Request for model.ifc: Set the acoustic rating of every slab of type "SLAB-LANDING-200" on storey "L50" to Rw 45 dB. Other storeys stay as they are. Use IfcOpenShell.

First a look at what the model holds.

```python
import ifcopenshell
import ifcopenshell.util.element

model = ifcopenshell.open("model.ifc")
print(model.schema)
storey = next(s for s in model.by_type("IfcBuildingStorey") if s.Name == "L50")
slabs = [e for e in ifcopenshell.util.element.get_decomposition(storey) if e.is_a("IfcSlab")]
seen = {}
for e in slabs:
    element_type = ifcopenshell.util.element.get_type(e)
    key = (element_type.Name if element_type != e and element_type else None, ifcopenshell.util.element.get_pset(e, "Pset_SlabCommon", "AcousticRating"))
    seen[key] = seen.get(key, 0) + 1
for (name, value), count in sorted(seen.items(), key=str):
    print(count, "x", name, "|", value)
```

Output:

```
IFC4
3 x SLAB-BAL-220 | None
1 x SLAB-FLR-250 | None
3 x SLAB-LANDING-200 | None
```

```python
import ifcopenshell
import ifcopenshell.api.pset
import ifcopenshell.util.element

model = ifcopenshell.open("model.ifc")

storey = next(s for s in model.by_type("IfcBuildingStorey") if s.Name == "L50")
slabs = [e for e in ifcopenshell.util.element.get_decomposition(storey) if e.is_a("IfcSlab")]

count = 0
for e in slabs:
    element_type = ifcopenshell.util.element.get_type(e)
    if element_type in (None, e) or element_type.Name != "SLAB-LANDING-200":
        continue
    found = ifcopenshell.util.element.get_pset(e, "Pset_SlabCommon", should_inherit=False)
    if found:
        pset = model.by_id(found["id"])
        if len(ifcopenshell.util.element.get_elements_by_pset(pset)) > 1:
            pset = ifcopenshell.api.pset.unshare_pset(model, products=[e], pset=pset)[0]
    else:
        pset = ifcopenshell.api.pset.add_pset(model, product=e, name="Pset_SlabCommon")
    ifcopenshell.api.pset.edit_pset(model, pset=pset, properties={"AcousticRating": "Rw 45 dB"})
    count += 1

print(count, "slabs updated")

model.write("model-out.ifc")
```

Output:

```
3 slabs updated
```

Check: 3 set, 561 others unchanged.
